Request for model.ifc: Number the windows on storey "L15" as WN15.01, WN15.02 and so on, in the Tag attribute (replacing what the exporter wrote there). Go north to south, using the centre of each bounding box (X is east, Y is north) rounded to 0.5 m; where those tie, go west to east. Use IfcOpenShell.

First a look at what the model holds.

```python
import ifcopenshell
import ifcopenshell.util.element
import ifcopenshell.util.placement

model = ifcopenshell.open("model.ifc")
print(model.schema)
storey = next(s for s in model.by_type("IfcBuildingStorey") if s.Name == "L15")
windows = [e for e in ifcopenshell.util.element.get_decomposition(storey) if e.is_a("IfcWindow")]
for e in sorted(windows, key=lambda e: e.id()):
    origin = ifcopenshell.util.placement.get_local_placement(e.ObjectPlacement)[:3, 3]
    print(e.id(), e.Tag, e.Name, origin.round(2) + 0.0, sep=" | ")
```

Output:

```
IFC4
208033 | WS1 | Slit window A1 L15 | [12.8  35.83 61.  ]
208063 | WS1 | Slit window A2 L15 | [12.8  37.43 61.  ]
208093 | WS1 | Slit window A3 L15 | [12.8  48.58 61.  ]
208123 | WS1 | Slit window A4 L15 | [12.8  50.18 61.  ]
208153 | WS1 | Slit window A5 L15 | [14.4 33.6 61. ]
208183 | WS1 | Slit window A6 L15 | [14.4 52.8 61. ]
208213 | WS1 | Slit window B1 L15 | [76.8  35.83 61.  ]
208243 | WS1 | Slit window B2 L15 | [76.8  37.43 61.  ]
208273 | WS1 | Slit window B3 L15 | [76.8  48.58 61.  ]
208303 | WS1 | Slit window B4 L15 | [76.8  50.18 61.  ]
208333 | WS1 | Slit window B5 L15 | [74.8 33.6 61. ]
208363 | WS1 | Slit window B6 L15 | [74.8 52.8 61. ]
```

```python
import ifcopenshell
import ifcopenshell.geom
import ifcopenshell.util.element
import ifcopenshell.util.shape

model = ifcopenshell.open("model.ifc")
settings = ifcopenshell.geom.settings()
settings.set("use-world-coords", True)


def centre(element):
    shape = ifcopenshell.geom.create_shape(settings, element)
    return ifcopenshell.util.shape.get_bbox_centroid(shape.geometry)


storey = next(s for s in model.by_type("IfcBuildingStorey") if s.Name == "L15")
windows = [e for e in ifcopenshell.util.element.get_decomposition(storey) if e.is_a("IfcWindow")]

# Insertion points can sit at a corner or the storey origin, so sort by the geometry (in metres).
centres = {e: centre(e) for e in windows}
windows.sort(key=lambda e: (-round(centres[e][1] / 0.5), centres[e][0]))

for i, e in enumerate(windows, start=1):
    number = f"WN15.{i:02d}"
    e.Tag = number
    print(e.id(), number)

model.write("model_edited.ifc")
```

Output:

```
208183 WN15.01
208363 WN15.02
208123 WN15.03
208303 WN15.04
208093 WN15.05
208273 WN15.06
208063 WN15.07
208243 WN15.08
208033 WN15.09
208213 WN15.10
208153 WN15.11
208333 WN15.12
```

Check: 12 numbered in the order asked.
